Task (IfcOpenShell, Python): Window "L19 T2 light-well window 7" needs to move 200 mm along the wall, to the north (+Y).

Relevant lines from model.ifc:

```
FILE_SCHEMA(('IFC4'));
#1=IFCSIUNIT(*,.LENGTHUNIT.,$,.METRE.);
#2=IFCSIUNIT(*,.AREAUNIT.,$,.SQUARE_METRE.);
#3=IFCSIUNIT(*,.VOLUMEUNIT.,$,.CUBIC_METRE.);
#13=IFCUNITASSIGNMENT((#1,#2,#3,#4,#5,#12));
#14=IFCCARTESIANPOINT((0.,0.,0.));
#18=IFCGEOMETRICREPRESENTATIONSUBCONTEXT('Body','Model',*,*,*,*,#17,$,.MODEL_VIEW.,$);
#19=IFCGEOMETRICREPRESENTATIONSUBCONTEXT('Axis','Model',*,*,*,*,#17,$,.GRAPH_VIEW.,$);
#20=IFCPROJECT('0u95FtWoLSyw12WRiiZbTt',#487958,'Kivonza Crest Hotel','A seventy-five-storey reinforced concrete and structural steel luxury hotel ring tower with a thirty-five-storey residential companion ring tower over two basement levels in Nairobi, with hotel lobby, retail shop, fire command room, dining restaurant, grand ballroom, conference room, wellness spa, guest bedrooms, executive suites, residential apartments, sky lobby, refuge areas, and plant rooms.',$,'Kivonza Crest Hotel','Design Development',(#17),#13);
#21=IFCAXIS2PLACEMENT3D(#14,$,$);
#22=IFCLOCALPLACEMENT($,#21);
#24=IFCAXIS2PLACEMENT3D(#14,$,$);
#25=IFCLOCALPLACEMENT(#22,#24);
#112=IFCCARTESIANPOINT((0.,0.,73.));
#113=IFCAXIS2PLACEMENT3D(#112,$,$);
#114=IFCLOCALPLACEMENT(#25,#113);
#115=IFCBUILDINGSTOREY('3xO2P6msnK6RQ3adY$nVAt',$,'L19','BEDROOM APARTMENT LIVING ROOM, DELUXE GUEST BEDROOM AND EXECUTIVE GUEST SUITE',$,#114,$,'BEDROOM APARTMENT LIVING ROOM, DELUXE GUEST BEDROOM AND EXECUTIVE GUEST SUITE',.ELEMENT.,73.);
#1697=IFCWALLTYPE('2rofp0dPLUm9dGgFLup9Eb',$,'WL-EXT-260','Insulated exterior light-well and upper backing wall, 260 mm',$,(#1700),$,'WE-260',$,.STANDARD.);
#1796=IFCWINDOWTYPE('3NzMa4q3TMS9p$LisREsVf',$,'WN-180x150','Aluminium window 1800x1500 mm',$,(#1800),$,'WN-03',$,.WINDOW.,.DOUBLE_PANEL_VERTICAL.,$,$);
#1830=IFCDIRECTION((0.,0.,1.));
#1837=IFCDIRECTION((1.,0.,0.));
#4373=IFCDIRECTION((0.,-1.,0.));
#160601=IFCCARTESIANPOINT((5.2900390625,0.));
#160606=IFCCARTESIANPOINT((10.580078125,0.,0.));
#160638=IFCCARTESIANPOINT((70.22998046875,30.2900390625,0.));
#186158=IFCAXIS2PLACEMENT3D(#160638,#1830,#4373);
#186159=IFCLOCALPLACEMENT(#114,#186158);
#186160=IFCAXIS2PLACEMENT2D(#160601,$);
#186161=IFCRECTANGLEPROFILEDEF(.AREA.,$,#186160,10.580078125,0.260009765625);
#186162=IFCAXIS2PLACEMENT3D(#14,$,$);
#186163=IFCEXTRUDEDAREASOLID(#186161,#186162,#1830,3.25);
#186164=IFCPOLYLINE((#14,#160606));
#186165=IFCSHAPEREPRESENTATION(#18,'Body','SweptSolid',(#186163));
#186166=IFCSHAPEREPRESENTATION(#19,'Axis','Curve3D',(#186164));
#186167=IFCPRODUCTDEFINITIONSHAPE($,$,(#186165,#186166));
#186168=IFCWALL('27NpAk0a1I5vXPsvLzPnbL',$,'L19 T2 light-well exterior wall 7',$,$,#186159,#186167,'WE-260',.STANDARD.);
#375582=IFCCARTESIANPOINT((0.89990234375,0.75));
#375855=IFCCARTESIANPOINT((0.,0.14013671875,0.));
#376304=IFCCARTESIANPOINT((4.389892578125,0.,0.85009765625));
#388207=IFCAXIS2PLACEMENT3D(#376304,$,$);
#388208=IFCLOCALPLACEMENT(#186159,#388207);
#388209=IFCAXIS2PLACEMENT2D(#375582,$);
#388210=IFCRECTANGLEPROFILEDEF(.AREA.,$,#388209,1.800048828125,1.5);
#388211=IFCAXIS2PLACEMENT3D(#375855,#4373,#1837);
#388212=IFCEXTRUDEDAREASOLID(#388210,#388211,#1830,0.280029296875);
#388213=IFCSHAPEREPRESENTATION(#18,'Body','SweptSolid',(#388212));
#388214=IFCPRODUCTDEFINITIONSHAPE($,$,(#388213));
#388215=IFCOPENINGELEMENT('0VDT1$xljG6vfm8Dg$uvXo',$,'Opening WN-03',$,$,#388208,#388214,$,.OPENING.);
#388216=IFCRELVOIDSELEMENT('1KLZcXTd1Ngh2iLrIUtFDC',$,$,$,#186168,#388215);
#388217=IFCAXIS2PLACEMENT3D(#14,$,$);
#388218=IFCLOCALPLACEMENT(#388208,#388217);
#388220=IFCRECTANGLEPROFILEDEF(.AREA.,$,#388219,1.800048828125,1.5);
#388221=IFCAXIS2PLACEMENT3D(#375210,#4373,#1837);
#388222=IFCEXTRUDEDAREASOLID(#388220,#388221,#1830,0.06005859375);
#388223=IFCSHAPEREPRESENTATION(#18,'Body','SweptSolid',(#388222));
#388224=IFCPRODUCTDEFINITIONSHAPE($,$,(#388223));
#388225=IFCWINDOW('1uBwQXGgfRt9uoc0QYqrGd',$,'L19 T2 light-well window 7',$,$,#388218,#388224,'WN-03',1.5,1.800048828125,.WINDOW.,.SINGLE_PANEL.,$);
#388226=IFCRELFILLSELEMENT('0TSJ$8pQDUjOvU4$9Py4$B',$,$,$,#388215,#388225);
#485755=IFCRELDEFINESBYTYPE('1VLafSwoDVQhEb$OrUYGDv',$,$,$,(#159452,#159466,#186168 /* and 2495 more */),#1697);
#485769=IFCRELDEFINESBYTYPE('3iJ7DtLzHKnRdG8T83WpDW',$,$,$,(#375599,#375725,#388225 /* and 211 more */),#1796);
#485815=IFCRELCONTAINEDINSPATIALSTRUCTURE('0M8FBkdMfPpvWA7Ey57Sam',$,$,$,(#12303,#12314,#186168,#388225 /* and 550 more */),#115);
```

```python
import ifcopenshell
import ifcopenshell.api.geometry
import ifcopenshell.util.placement
import ifcopenshell.util.unit

model = ifcopenshell.open("model.ifc")
unit_scale = ifcopenshell.util.unit.calculate_unit_scale(model)

window = model.by_guid("1uBwQXGgfRt9uoc0QYqrGd")
opening = window.FillsVoids[0].RelatingOpeningElement
wall = opening.VoidsElements[0].RelatingBuildingElement

wall_matrix = ifcopenshell.util.placement.get_local_placement(wall.ObjectPlacement)
shift = wall_matrix[:3, 0] * -0.2 / unit_scale
before = ifcopenshell.util.placement.get_local_placement(window.ObjectPlacement)[:3, 3].copy()

# The window is placed relative to its opening, so it follows when the opening moves.
matrix = ifcopenshell.util.placement.get_local_placement(opening.ObjectPlacement)
matrix[:3, 3] += shift
ifcopenshell.api.geometry.edit_object_placement(
    model, product=opening, matrix=matrix, is_si=False, should_transform_children=True
)

after = ifcopenshell.util.placement.get_local_placement(window.ObjectPlacement)[:3, 3]
print("window moved by", (after - before).round(3) + 0.0)

model.write("model_updated.ifc")
```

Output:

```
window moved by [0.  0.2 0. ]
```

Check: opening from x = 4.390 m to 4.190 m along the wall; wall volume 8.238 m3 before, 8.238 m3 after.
